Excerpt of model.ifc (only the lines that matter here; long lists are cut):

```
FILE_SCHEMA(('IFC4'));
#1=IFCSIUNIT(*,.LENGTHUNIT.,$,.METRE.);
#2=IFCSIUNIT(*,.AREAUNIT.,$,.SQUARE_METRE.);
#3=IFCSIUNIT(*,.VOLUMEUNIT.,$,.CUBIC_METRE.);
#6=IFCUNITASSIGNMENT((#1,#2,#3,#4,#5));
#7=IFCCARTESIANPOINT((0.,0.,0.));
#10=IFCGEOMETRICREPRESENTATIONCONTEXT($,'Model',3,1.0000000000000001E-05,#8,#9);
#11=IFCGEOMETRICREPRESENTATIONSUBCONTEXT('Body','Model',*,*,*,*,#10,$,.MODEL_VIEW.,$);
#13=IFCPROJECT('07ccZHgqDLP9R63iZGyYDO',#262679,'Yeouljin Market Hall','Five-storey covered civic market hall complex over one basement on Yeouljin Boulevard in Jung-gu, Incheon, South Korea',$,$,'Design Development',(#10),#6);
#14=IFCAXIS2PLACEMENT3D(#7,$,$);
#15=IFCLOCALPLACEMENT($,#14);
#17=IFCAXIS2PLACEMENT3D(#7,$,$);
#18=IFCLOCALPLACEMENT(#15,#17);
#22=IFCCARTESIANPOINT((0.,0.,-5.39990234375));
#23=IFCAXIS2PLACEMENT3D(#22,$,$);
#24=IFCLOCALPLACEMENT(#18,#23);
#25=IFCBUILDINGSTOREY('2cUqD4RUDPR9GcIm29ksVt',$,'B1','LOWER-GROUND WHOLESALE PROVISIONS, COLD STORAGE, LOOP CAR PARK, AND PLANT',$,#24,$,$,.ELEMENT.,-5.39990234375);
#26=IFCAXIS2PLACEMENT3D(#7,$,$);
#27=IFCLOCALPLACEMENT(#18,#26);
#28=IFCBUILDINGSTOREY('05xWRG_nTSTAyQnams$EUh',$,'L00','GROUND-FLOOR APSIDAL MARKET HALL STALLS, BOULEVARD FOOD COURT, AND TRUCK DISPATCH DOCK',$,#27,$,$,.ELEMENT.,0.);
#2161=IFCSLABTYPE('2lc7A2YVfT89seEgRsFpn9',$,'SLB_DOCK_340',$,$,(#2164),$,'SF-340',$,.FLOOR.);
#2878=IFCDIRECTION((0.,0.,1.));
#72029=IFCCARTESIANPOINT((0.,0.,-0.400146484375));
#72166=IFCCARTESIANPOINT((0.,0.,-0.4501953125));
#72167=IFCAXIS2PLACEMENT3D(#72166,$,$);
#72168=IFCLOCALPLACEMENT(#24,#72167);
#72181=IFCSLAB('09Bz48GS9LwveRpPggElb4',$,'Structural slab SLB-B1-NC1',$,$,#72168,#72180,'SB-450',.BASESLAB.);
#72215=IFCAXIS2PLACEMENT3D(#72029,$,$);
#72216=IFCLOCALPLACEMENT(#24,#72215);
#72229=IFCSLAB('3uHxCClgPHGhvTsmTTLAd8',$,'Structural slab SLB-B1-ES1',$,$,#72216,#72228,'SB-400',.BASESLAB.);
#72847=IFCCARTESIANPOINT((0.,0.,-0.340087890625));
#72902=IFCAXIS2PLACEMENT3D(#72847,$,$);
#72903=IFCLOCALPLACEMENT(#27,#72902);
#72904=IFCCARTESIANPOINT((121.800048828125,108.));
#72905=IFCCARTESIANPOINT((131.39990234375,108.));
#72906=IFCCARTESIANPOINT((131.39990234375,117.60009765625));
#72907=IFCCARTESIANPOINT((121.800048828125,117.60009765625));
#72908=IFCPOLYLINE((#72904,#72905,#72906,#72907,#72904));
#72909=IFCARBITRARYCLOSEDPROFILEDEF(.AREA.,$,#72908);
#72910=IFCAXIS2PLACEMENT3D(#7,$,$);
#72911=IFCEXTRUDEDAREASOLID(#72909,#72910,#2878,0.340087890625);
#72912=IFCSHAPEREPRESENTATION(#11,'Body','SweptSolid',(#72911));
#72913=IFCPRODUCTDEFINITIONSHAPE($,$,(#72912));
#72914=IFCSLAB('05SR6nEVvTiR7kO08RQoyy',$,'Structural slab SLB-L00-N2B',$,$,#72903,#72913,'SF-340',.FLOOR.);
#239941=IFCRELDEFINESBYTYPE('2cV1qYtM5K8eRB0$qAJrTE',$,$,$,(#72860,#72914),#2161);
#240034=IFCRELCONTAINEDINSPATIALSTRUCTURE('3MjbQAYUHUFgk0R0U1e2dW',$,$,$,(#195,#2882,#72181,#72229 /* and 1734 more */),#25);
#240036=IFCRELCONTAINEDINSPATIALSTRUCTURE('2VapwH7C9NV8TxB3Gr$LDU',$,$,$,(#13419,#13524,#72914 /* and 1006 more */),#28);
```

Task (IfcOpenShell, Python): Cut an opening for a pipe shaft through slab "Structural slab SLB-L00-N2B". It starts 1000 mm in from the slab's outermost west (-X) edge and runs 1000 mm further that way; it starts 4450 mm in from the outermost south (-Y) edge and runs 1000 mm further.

```python
import numpy as np
import ifcopenshell
import ifcopenshell.api.feature
import ifcopenshell.api.geometry
import ifcopenshell.api.root
import ifcopenshell.geom
import ifcopenshell.util.placement
import ifcopenshell.util.representation
import ifcopenshell.util.shape
import ifcopenshell.util.unit

model = ifcopenshell.open("model.ifc")
unit_scale = ifcopenshell.util.unit.calculate_unit_scale(model)
settings = ifcopenshell.geom.settings()


def volume(element):
    """Net volume in cubic metres, openings subtracted."""
    shape = ifcopenshell.geom.create_shape(settings, element)
    return ifcopenshell.util.shape.get_volume(shape.geometry)


slab = model.by_guid("05SR6nEVvTiR7kO08RQoyy")
before = volume(slab)

# Extent in the slab's own axes, in metres. The edges named are its -X and -Y sides.
slab_shape = ifcopenshell.geom.create_shape(settings, slab)
vertices = ifcopenshell.util.shape.get_vertices(slab_shape.geometry)
x_min, y_min, bottom = vertices.min(axis=0)
top = vertices[:, 2].max()

opening = ifcopenshell.api.root.create_entity(model, ifc_class="IfcOpeningElement", name="Pipe shaft opening", predefined_type="OPENING")
context = ifcopenshell.util.representation.get_context(model, "Model", "Body", "MODEL_VIEW")
width, depth = 1, 1
outline = [(0.0, 0.0), (width, 0.0), (width, depth), (0.0, depth), (0.0, 0.0)]
# Overshoot both faces by 50 mm so the cut is clean.
shape = ifcopenshell.api.geometry.add_slab_representation(
    model, context=context, depth=top - bottom + 0.1, polyline=outline
)
ifcopenshell.api.geometry.assign_representation(model, product=opening, representation=shape)

matrix = ifcopenshell.util.placement.get_local_placement(slab.ObjectPlacement)
matrix[:, 3] = matrix @ np.append(np.array([x_min + 1, y_min + 4.45, bottom - 0.05]) / unit_scale, 1.0)
ifcopenshell.api.geometry.edit_object_placement(model, product=opening, matrix=matrix, is_si=False)
ifcopenshell.api.feature.add_feature(model, feature=opening, element=slab)

after = volume(slab)

print(f"slab volume {before:.3f} -> {after:.3f} m3")

model.write("model_rev.ifc")
```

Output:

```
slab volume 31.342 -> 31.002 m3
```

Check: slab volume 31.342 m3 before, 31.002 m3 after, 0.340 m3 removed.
